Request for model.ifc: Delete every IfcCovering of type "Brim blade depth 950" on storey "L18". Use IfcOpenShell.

First a look at what the model holds.

```python
import ifcopenshell
import ifcopenshell.util.element

model = ifcopenshell.open("model.ifc")
print(model.schema)
storey = next(s for s in model.by_type("IfcBuildingStorey") if s.Name == "L18")
coverings = [e for e in ifcopenshell.util.element.get_decomposition(storey) if e.is_a("IfcCovering")]
seen = {}
for e in coverings:
    element_type = ifcopenshell.util.element.get_type(e)
    name = element_type.Name if element_type not in (None, e) else None
    seen[name] = seen.get(name, 0) + 1
for name, count in sorted(seen.items(), key=str):
    print(count, "x", name)
```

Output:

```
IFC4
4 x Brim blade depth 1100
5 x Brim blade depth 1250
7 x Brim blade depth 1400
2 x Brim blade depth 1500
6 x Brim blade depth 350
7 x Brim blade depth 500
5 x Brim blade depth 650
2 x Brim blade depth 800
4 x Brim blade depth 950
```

```python
import ifcopenshell
import ifcopenshell.api.root
import ifcopenshell.util.element

model = ifcopenshell.open("model.ifc")

storey = next(s for s in model.by_type("IfcBuildingStorey") if s.Name == "L18")
coverings = [e for e in ifcopenshell.util.element.get_decomposition(storey) if e.is_a("IfcCovering")]
targets = [e for e in coverings if (t := ifcopenshell.util.element.get_type(e)) not in (None, e) and t.Name == "Brim blade depth 950"]

for e in targets:
    ifcopenshell.api.root.remove_product(model, product=e)
print(len(targets), "removed")

model.write("model_edited.ifc")
```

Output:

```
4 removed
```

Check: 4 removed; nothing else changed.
